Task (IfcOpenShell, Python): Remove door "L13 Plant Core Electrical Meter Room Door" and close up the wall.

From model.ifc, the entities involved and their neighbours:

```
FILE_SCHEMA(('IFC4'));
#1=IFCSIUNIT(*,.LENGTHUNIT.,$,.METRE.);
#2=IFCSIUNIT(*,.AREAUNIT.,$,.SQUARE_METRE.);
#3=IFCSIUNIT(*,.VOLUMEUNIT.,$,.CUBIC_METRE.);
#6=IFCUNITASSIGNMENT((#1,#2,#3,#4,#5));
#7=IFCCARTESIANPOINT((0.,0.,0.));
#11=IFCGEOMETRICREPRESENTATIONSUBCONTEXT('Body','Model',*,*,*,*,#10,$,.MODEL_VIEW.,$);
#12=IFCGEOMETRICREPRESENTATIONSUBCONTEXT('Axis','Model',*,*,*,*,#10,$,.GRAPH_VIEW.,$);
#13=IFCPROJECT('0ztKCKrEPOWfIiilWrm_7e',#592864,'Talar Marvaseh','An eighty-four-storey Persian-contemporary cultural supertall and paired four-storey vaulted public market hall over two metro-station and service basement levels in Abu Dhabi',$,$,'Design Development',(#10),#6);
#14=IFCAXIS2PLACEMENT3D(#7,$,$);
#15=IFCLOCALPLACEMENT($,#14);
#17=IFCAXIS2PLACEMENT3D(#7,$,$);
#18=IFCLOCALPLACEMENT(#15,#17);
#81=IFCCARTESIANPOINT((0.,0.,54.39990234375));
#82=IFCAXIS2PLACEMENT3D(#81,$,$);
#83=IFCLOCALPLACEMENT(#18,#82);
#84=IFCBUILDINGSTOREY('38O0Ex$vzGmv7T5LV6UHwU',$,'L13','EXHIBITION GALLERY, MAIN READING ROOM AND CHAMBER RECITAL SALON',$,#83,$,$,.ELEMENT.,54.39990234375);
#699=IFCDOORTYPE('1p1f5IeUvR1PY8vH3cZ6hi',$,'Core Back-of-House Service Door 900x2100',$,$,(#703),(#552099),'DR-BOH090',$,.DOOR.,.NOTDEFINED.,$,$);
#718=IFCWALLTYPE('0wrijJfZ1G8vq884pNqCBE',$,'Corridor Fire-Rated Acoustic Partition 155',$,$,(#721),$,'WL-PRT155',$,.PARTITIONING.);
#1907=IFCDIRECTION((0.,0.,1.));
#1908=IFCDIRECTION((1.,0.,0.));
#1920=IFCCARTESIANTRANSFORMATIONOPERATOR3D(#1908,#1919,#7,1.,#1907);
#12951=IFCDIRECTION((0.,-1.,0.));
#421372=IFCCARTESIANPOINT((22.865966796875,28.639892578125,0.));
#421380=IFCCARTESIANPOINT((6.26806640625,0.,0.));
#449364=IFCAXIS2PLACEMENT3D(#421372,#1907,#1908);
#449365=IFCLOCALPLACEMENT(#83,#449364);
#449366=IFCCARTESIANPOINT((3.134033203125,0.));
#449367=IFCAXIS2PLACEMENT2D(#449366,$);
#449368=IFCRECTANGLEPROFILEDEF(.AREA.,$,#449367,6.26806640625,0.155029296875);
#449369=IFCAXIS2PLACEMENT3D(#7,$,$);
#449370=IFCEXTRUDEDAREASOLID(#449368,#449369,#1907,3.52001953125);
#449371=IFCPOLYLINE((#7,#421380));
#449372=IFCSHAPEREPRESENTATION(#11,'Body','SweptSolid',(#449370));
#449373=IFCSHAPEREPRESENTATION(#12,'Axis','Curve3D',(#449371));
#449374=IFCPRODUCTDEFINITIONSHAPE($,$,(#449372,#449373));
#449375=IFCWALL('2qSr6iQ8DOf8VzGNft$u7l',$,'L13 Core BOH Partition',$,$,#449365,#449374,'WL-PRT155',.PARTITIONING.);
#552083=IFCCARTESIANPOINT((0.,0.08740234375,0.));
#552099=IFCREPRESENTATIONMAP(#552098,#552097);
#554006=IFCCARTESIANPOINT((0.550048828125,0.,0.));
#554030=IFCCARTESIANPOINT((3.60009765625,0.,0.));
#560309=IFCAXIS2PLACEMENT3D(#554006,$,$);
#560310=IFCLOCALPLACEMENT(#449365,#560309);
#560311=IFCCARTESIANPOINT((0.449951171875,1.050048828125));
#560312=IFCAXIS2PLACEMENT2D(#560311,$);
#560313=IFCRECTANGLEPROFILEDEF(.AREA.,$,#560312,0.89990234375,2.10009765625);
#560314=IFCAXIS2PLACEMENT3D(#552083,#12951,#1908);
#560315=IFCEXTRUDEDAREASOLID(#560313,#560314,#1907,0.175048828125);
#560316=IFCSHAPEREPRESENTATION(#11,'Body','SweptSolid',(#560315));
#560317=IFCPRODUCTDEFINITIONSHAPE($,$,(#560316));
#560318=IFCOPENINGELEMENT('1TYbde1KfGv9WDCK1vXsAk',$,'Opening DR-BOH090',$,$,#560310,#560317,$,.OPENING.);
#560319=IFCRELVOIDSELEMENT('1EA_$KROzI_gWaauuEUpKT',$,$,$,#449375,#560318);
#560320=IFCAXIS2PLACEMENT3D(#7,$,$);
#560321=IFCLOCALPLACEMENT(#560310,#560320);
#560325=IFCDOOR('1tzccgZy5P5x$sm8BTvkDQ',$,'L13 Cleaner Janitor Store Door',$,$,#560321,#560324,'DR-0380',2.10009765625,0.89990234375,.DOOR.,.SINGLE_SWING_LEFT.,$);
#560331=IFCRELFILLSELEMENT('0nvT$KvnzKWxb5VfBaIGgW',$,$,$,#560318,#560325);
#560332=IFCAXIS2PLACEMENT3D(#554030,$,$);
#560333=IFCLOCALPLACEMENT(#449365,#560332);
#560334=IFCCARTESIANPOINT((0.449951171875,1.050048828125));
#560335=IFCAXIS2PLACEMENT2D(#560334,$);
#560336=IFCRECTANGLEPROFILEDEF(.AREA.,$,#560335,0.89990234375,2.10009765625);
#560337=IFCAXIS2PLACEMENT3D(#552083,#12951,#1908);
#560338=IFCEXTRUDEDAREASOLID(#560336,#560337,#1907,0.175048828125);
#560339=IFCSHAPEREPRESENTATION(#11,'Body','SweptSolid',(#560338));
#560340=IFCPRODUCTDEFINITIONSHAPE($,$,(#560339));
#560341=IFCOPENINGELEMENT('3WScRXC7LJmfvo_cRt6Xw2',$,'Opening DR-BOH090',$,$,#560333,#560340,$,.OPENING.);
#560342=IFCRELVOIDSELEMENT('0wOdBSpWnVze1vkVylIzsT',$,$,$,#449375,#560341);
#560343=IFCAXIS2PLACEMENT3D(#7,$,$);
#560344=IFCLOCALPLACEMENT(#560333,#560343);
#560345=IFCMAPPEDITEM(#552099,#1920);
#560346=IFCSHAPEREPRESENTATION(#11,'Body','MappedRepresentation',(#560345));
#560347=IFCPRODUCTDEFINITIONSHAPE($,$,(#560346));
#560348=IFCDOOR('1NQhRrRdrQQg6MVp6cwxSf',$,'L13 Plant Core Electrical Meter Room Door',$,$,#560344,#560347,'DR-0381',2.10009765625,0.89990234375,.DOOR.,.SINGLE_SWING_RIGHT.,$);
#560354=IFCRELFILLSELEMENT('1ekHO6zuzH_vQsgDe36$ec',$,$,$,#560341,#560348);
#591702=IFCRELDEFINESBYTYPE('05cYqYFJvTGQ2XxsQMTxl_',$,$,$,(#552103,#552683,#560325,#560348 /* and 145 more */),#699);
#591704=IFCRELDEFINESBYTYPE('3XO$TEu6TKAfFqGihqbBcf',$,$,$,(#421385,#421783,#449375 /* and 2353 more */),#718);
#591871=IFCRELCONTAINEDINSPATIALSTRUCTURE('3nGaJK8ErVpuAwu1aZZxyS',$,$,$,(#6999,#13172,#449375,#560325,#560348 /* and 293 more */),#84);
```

```python
import ifcopenshell
import ifcopenshell.api.feature
import ifcopenshell.api.root
import ifcopenshell.geom
import ifcopenshell.util.shape

model = ifcopenshell.open("model.ifc")
settings = ifcopenshell.geom.settings()


def volume(element):
    """Net volume in cubic metres, openings subtracted."""
    shape = ifcopenshell.geom.create_shape(settings, element)
    return ifcopenshell.util.shape.get_volume(shape.geometry)


door = model.by_id(560348)
opening = door.FillsVoids[0].RelatingOpeningElement
wall = opening.VoidsElements[0].RelatingBuildingElement
before = volume(wall)

ifcopenshell.api.root.remove_product(model, product=door)
ifcopenshell.api.feature.remove_feature(model, feature=opening)

after = volume(wall)

print(f"wall volume {before:.3f} -> {after:.3f} m3")

model.write("model_rev.ifc")
```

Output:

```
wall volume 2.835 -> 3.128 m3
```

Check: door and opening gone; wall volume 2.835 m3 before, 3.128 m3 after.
